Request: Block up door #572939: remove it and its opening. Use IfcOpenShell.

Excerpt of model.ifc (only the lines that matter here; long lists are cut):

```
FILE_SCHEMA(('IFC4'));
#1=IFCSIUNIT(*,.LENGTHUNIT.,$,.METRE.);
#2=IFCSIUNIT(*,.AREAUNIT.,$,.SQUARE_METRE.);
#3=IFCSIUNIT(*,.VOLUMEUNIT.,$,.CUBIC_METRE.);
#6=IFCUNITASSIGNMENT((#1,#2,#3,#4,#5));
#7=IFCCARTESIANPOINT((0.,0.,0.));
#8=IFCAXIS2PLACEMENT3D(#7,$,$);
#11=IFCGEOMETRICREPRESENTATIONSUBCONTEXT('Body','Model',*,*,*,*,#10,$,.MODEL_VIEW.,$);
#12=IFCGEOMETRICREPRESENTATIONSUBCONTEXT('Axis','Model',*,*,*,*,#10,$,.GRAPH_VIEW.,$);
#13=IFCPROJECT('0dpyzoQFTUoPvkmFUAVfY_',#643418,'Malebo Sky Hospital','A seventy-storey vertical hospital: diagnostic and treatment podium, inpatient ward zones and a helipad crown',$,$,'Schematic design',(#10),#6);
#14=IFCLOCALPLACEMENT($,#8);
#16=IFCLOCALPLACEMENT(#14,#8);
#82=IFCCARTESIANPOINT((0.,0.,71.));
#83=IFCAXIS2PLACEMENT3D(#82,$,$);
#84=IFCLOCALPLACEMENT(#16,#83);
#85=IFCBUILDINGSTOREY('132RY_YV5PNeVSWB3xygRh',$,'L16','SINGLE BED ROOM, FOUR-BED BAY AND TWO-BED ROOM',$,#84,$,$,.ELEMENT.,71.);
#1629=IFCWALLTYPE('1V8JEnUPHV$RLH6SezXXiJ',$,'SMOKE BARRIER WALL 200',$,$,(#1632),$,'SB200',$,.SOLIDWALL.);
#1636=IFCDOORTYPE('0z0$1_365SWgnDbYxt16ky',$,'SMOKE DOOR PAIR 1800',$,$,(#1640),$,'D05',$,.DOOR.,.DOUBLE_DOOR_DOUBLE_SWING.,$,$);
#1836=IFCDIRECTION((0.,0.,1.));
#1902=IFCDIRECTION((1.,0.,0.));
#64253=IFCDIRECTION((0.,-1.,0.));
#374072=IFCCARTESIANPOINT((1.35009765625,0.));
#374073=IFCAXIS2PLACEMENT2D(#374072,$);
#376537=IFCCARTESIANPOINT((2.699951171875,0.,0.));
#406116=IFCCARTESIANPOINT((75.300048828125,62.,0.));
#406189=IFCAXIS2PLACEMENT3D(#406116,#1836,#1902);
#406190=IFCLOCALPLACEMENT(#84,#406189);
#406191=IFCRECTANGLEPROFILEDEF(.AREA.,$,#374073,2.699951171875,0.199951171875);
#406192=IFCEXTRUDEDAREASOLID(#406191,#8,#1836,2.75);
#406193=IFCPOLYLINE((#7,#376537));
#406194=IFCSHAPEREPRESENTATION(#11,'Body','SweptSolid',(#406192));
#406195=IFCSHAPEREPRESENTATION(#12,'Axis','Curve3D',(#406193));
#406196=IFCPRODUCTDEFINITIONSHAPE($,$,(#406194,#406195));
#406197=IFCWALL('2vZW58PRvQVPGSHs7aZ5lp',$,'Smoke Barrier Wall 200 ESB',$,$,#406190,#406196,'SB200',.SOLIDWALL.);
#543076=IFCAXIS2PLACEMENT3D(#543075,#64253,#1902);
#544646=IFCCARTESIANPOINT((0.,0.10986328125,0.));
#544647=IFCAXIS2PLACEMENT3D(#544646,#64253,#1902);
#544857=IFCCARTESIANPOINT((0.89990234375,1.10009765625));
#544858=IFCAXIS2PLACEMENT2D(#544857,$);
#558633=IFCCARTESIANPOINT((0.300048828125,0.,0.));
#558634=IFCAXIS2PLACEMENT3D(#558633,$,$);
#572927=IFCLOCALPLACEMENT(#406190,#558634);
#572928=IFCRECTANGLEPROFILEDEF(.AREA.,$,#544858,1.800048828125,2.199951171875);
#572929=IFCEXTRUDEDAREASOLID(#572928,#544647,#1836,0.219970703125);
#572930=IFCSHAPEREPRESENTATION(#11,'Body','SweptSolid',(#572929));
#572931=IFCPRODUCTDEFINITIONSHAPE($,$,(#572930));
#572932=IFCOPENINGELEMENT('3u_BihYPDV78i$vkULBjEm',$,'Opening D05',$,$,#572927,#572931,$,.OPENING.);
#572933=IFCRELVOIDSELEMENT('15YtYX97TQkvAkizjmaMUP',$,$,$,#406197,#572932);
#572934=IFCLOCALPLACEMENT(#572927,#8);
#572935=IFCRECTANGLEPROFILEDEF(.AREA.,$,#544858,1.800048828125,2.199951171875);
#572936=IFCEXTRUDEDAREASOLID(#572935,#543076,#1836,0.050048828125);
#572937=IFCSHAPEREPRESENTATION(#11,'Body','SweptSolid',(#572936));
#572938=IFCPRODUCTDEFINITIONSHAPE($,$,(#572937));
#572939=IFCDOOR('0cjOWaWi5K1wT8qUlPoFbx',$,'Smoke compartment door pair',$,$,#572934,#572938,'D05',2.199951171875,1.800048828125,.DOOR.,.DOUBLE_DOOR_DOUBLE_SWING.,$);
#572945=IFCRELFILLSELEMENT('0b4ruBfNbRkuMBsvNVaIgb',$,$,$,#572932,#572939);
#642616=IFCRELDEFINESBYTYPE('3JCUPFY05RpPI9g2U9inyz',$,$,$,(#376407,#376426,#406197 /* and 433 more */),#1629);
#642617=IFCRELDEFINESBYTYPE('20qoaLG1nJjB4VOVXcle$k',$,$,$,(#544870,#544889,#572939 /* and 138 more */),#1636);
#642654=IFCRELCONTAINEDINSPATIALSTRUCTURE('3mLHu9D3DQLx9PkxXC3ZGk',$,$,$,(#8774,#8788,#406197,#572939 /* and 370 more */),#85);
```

```python
import ifcopenshell
import ifcopenshell.api.feature
import ifcopenshell.api.root
import ifcopenshell.geom
import ifcopenshell.util.shape

model = ifcopenshell.open("model.ifc")
settings = ifcopenshell.geom.settings()


def volume(element):
    """Net volume in cubic metres, openings subtracted."""
    shape = ifcopenshell.geom.create_shape(settings, element)
    return ifcopenshell.util.shape.get_volume(shape.geometry)


door = model.by_guid("0cjOWaWi5K1wT8qUlPoFbx")
opening = door.FillsVoids[0].RelatingOpeningElement
wall = opening.VoidsElements[0].RelatingBuildingElement
before = volume(wall)

ifcopenshell.api.root.remove_product(model, product=door)
ifcopenshell.api.feature.remove_feature(model, feature=opening)

after = volume(wall)

print(f"wall volume {before:.3f} -> {after:.3f} m3")

model.write("model-out.ifc")
```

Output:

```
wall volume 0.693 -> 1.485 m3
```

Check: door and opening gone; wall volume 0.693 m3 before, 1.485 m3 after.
